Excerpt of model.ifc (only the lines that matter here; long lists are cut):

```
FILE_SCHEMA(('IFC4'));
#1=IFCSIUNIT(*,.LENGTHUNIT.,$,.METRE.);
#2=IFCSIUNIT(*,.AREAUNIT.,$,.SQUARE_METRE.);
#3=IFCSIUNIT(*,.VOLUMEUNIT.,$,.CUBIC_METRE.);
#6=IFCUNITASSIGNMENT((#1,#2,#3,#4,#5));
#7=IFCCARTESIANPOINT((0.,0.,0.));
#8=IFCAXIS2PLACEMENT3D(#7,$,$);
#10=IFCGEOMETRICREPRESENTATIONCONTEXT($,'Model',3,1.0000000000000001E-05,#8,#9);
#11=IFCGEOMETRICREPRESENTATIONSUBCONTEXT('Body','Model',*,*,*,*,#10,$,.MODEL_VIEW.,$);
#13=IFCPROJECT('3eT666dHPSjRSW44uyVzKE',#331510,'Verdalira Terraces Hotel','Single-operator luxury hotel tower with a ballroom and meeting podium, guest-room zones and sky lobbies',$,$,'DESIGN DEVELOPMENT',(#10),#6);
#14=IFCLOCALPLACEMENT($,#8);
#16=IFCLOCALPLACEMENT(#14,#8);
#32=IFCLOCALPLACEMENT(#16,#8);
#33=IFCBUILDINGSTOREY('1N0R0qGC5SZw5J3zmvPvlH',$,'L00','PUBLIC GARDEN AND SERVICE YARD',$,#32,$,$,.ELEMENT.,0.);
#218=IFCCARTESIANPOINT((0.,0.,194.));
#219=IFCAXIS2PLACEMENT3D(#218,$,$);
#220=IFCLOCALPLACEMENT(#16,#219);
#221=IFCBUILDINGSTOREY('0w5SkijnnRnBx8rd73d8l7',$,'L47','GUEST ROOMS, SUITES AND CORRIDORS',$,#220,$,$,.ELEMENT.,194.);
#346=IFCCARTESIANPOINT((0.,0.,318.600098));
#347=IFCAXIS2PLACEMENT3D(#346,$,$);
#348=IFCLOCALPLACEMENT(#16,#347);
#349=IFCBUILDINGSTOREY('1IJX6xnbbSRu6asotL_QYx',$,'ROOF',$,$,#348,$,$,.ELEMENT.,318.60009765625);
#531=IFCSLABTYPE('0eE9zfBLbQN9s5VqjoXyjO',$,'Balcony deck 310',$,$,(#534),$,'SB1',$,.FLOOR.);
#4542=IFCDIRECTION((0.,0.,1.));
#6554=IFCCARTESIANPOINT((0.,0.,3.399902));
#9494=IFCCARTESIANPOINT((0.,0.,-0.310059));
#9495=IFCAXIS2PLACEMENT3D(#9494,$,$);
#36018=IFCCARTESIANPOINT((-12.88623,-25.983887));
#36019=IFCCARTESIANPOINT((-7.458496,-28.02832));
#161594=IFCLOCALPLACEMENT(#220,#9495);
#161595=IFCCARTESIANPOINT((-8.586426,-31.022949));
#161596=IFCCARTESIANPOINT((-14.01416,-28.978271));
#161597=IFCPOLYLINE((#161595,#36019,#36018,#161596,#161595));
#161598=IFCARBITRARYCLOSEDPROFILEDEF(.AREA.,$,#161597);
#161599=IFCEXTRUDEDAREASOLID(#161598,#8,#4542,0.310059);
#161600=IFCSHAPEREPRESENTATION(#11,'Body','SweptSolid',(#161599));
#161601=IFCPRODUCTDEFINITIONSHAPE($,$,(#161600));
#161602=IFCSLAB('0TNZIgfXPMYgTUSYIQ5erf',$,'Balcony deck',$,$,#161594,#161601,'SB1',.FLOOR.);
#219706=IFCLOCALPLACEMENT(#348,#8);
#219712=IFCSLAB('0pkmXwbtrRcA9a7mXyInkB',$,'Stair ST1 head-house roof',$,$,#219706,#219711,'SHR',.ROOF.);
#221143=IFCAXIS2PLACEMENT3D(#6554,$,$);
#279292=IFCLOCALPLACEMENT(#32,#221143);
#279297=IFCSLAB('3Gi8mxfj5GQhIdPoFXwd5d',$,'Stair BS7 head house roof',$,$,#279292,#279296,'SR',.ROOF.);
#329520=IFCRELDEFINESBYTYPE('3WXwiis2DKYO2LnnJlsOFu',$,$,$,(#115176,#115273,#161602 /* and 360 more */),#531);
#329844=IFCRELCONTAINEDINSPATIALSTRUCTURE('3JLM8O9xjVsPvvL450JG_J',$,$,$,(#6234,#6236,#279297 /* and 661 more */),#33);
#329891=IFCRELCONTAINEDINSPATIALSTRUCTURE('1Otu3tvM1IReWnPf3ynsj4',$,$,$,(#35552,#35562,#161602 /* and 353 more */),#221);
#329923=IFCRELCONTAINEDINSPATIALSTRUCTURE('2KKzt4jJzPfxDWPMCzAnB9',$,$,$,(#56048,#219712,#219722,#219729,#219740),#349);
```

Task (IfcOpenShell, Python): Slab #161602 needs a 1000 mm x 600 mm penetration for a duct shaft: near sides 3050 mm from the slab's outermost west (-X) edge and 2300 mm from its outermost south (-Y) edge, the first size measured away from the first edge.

```python
import numpy as np
import ifcopenshell
import ifcopenshell.api.feature
import ifcopenshell.api.geometry
import ifcopenshell.api.root
import ifcopenshell.geom
import ifcopenshell.util.placement
import ifcopenshell.util.representation
import ifcopenshell.util.shape
import ifcopenshell.util.unit

model = ifcopenshell.open("model.ifc")
unit_scale = ifcopenshell.util.unit.calculate_unit_scale(model)
settings = ifcopenshell.geom.settings()


def volume(element):
    """Net volume in cubic metres, openings subtracted."""
    shape = ifcopenshell.geom.create_shape(settings, element)
    return ifcopenshell.util.shape.get_volume(shape.geometry)


slab = model.by_guid("0TNZIgfXPMYgTUSYIQ5erf")
before = volume(slab)

# Extent in the slab's own axes, in metres. The edges named are its -X and -Y sides.
slab_shape = ifcopenshell.geom.create_shape(settings, slab)
vertices = ifcopenshell.util.shape.get_vertices(slab_shape.geometry)
x_min, y_min, bottom = vertices.min(axis=0)
top = vertices[:, 2].max()

opening = ifcopenshell.api.root.create_entity(model, ifc_class="IfcOpeningElement", name="Duct shaft opening", predefined_type="OPENING")
context = ifcopenshell.util.representation.get_context(model, "Model", "Body", "MODEL_VIEW")
width, depth = 1, 0.6
outline = [(0.0, 0.0), (width, 0.0), (width, depth), (0.0, depth), (0.0, 0.0)]
# Overshoot both faces by 50 mm so the cut is clean.
shape = ifcopenshell.api.geometry.add_slab_representation(
    model, context=context, depth=top - bottom + 0.1, polyline=outline
)
ifcopenshell.api.geometry.assign_representation(model, product=opening, representation=shape)

matrix = ifcopenshell.util.placement.get_local_placement(slab.ObjectPlacement)
matrix[:, 3] = matrix @ np.append(np.array([x_min + 3.05, y_min + 2.3, bottom - 0.05]) / unit_scale, 1.0)
ifcopenshell.api.geometry.edit_object_placement(model, product=opening, matrix=matrix, is_si=False)
ifcopenshell.api.feature.add_feature(model, feature=opening, element=slab)

after = volume(slab)

print(f"slab volume {before:.3f} -> {after:.3f} m3")

model.write("model_updated.ifc")
```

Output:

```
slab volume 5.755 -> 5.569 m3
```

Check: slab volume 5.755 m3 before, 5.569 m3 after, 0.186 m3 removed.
